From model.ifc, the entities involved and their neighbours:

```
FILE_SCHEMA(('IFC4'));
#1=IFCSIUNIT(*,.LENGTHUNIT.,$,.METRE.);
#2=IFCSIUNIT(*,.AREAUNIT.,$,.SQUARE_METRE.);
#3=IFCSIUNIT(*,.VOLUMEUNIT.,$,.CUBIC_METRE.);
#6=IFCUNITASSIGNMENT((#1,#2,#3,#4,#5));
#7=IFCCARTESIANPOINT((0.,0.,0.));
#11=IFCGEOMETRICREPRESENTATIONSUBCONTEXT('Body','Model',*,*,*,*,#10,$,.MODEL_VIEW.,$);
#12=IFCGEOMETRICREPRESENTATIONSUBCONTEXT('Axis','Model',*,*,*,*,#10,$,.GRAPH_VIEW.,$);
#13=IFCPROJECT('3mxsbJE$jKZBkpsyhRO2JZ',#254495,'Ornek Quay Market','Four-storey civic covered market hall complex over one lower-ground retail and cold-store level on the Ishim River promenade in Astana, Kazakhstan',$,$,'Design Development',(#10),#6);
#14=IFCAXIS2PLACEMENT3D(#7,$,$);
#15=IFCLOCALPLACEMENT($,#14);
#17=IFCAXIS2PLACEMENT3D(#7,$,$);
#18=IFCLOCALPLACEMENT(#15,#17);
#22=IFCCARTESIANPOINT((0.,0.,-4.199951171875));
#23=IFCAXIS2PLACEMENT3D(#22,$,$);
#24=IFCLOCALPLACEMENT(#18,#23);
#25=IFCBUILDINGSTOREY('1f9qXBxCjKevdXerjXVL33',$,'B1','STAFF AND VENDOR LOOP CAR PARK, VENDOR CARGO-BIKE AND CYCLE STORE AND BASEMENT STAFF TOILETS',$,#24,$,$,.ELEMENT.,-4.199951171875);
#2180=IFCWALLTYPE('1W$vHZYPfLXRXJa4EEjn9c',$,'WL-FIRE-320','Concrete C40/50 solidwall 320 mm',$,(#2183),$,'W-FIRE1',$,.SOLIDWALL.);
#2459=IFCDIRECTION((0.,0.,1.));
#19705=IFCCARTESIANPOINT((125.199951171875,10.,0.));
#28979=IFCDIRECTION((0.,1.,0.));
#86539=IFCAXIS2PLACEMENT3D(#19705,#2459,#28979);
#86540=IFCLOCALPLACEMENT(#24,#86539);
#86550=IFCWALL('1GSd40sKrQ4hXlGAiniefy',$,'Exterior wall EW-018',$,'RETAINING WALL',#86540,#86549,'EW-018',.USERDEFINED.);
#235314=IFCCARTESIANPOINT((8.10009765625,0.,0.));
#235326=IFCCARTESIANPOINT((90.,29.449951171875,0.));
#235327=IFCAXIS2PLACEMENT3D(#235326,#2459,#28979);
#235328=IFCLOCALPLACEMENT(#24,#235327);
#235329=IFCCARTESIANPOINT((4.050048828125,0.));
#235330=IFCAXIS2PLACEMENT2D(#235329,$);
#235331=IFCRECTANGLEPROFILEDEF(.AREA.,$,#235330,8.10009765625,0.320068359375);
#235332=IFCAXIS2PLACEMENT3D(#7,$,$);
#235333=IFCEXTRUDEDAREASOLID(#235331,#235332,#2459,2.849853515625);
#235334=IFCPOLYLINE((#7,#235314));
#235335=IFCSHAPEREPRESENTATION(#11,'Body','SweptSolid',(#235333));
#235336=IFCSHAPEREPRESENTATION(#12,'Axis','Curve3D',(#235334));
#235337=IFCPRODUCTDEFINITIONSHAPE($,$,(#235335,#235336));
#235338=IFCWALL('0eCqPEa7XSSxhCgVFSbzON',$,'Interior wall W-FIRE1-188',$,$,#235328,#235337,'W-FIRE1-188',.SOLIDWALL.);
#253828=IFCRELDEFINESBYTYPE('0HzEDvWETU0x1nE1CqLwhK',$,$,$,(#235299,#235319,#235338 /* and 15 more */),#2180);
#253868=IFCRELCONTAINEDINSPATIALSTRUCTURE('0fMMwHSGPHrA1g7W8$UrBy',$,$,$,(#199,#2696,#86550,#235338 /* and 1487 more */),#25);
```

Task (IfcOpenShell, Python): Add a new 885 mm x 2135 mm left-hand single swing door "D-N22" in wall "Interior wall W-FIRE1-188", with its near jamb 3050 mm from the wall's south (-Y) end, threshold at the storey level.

```python
import numpy as np
import ifcopenshell
import ifcopenshell.api.feature
import ifcopenshell.api.geometry
import ifcopenshell.api.root
import ifcopenshell.api.spatial
import ifcopenshell.geom
import ifcopenshell.util.element
import ifcopenshell.util.placement
import ifcopenshell.util.representation
import ifcopenshell.util.shape
import ifcopenshell.util.unit

model = ifcopenshell.open("model.ifc")
unit_scale = ifcopenshell.util.unit.calculate_unit_scale(model)
settings = ifcopenshell.geom.settings()


def volume(element):
    """Net volume in cubic metres, openings subtracted."""
    shape = ifcopenshell.geom.create_shape(settings, element)
    return ifcopenshell.util.shape.get_volume(shape.geometry)


wall = model.by_guid("0eCqPEa7XSSxhCgVFSbzON")
storey = ifcopenshell.util.element.get_container(wall, ifc_class="IfcBuildingStorey")
context = ifcopenshell.util.representation.get_context(model, "Model", "Body", "MODEL_VIEW")
before = volume(wall)

width, height, from_end, sill = 0.885, 2.135, 3.05, 0.0  # metres

# The wall runs along its own X axis, and the end named is its -X end.
wall_shape = ifcopenshell.geom.create_shape(settings, wall)
x, y, z = ifcopenshell.util.shape.get_vertices(wall_shape.geometry).T
start = x.min() + from_end
face, thickness = float(y.min()), float(y.max() - y.min())
wall_matrix = ifcopenshell.util.placement.get_local_placement(wall.ObjectPlacement)
level = ifcopenshell.util.placement.get_local_placement(storey.ObjectPlacement)[2, 3]


def in_wall(x, y):
    """Placement at x, y metres in the wall's axes, at sill height."""
    matrix = wall_matrix.copy()
    matrix[:, 3] = wall_matrix @ np.array([x / unit_scale, y / unit_scale, 0.0, 1.0])
    matrix[2, 3] = level + sill / unit_scale
    return matrix


# Opening: a box that overshoots both wall faces by 50 mm.
opening = ifcopenshell.api.root.create_entity(model, ifc_class="IfcOpeningElement", predefined_type="OPENING")
box = ifcopenshell.api.geometry.add_wall_representation(
    model, context=context, length=width, height=height, thickness=thickness + 0.1
)
ifcopenshell.api.geometry.assign_representation(model, product=opening, representation=box)
ifcopenshell.api.geometry.edit_object_placement(model, product=opening, matrix=in_wall(start, face - 0.05), is_si=False)
ifcopenshell.api.feature.add_feature(model, feature=opening, element=wall)

door = ifcopenshell.api.root.create_entity(model, ifc_class="IfcDoor", name="D-N22", predefined_type="DOOR")
door.OverallWidth, door.OverallHeight = width / unit_scale, height / unit_scale
door.OperationType = "SINGLE_SWING_LEFT"
body = ifcopenshell.api.geometry.add_door_representation(
    model,
    context=context,
    overall_width=door.OverallWidth,
    overall_height=door.OverallHeight,
    operation_type="SINGLE_SWING_LEFT",
    lining_properties={"LiningDepth": thickness / unit_scale, "ThresholdDepth": thickness / unit_scale},
)
ifcopenshell.api.geometry.assign_representation(model, product=door, representation=body)
ifcopenshell.api.spatial.assign_container(model, products=[door], relating_structure=storey)
ifcopenshell.api.feature.add_filling(model, opening=opening, element=door)

# The lining spans the wall, so the door starts at the wall face.
ifcopenshell.api.geometry.edit_object_placement(model, product=door, matrix=in_wall(start, face), is_si=False)

after = volume(wall)

print(f"wall volume {before:.3f} -> {after:.3f} m3")

model.write("model-out.ifc")
```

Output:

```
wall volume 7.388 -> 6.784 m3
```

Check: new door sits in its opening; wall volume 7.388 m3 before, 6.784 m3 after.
